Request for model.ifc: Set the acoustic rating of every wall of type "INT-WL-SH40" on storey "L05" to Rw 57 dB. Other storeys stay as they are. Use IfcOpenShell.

First a look at what the model holds.

```python
import ifcopenshell
import ifcopenshell.util.element

model = ifcopenshell.open("model.ifc")
print(model.schema)
storey = next(s for s in model.by_type("IfcBuildingStorey") if s.Name == "L05")
walls = [e for e in ifcopenshell.util.element.get_decomposition(storey) if e.is_a("IfcWall")]
seen = {}
for e in walls:
    element_type = ifcopenshell.util.element.get_type(e)
    key = (element_type.Name if element_type != e and element_type else None, ifcopenshell.util.element.get_pset(e, "Pset_WallCommon", "AcousticRating"))
    seen[key] = seen.get(key, 0) + 1
for (name, value), count in sorted(seen.items(), key=str):
    print(count, "x", name, "|", value)
```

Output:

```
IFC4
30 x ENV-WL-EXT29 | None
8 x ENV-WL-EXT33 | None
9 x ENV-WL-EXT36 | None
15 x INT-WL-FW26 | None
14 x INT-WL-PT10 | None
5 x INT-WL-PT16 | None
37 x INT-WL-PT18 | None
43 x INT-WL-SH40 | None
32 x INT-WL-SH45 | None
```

```python
import ifcopenshell
import ifcopenshell.api.pset
import ifcopenshell.util.element

model = ifcopenshell.open("model.ifc")

storey = next(s for s in model.by_type("IfcBuildingStorey") if s.Name == "L05")
walls = [e for e in ifcopenshell.util.element.get_decomposition(storey) if e.is_a("IfcWall")]

count = 0
for e in walls:
    element_type = ifcopenshell.util.element.get_type(e)
    if element_type in (None, e) or element_type.Name != "INT-WL-SH40":
        continue
    # add_pset returns the element's existing set when there is one.
    pset = ifcopenshell.api.pset.add_pset(model, product=e, name="Pset_WallCommon")
    ifcopenshell.api.pset.edit_pset(model, pset=pset, properties={"AcousticRating": "Rw 57 dB"})
    count += 1

print(count, "walls updated")

model.write("model-out.ifc")
```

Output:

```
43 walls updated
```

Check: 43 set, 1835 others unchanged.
